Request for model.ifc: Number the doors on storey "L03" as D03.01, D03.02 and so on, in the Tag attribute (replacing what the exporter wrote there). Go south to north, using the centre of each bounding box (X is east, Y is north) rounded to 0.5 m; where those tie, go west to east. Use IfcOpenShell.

First a look at what the model holds.

```python
import ifcopenshell
import ifcopenshell.util.element
import ifcopenshell.util.placement

model = ifcopenshell.open("model.ifc")
print(model.schema)
storey = next(s for s in model.by_type("IfcBuildingStorey") if s.Name == "L03")
doors = [e for e in ifcopenshell.util.element.get_decomposition(storey) if e.is_a("IfcDoor")]
for e in sorted(doors, key=lambda e: e.id()):
    origin = ifcopenshell.util.placement.get_local_placement(e.ObjectPlacement)[:3, 3]
    print(e.id(), e.Tag, e.Name, origin.round(2) + 0.0, sep=" | ")
```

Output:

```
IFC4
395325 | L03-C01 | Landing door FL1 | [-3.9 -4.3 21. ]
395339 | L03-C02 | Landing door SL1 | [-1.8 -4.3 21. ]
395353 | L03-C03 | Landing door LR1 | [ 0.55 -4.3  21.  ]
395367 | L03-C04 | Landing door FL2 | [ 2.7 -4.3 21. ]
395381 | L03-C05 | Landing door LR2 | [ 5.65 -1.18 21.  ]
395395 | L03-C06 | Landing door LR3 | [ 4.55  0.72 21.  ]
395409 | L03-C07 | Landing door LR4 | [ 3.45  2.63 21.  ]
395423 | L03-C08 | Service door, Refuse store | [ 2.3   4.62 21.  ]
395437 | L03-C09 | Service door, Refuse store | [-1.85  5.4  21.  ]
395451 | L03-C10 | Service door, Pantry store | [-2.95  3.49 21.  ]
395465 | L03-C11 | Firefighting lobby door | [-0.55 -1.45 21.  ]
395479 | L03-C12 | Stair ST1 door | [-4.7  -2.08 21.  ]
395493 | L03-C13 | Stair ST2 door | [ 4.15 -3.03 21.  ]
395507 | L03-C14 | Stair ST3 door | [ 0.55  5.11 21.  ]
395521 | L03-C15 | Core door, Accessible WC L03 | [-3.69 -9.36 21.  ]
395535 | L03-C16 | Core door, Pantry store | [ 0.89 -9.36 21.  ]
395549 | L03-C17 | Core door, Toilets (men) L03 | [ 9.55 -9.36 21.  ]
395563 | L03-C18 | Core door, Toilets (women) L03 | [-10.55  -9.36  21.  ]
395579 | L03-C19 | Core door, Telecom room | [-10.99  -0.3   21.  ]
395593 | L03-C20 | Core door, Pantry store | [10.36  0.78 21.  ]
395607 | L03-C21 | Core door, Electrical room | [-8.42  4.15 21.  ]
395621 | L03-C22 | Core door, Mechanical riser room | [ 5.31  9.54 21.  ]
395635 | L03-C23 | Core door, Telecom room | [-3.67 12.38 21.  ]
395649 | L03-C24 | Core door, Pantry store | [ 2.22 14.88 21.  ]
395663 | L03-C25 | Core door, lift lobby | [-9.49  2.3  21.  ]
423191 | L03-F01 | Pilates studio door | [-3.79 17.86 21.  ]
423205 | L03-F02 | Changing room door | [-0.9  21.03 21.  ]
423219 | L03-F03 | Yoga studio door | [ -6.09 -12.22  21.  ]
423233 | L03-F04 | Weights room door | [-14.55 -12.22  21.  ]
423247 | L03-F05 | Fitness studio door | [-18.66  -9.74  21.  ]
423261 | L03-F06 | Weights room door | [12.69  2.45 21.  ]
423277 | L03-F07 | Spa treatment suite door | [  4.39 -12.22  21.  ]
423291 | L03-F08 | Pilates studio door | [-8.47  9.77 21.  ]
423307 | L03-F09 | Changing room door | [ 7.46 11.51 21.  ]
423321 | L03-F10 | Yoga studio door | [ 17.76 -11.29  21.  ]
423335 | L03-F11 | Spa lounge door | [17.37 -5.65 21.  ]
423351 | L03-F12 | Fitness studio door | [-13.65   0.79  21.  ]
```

```python
import ifcopenshell
import ifcopenshell.geom
import ifcopenshell.util.element
import ifcopenshell.util.shape

model = ifcopenshell.open("model.ifc")
settings = ifcopenshell.geom.settings()
settings.set("use-world-coords", True)


def centre(element):
    shape = ifcopenshell.geom.create_shape(settings, element)
    return ifcopenshell.util.shape.get_bbox_centroid(shape.geometry)


storey = next(s for s in model.by_type("IfcBuildingStorey") if s.Name == "L03")
doors = [e for e in ifcopenshell.util.element.get_decomposition(storey) if e.is_a("IfcDoor")]

# Insertion points can sit at a corner or the storey origin, so sort by the geometry (in metres).
centres = {e: centre(e) for e in doors}
doors.sort(key=lambda e: (round(centres[e][1] / 0.5), centres[e][0]))

for i, e in enumerate(doors, start=1):
    number = f"D03.{i:02d}"
    e.Tag = number
    print(e.id(), number)

model.write("model_edited.ifc")
```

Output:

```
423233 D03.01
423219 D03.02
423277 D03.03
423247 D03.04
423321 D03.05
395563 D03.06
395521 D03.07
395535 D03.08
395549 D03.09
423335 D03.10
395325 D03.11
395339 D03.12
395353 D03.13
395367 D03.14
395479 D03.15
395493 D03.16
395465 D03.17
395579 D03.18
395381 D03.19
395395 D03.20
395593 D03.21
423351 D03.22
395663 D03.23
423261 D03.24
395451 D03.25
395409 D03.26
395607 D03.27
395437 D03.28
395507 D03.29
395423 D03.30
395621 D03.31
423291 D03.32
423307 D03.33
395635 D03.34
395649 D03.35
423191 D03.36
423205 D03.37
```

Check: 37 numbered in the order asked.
